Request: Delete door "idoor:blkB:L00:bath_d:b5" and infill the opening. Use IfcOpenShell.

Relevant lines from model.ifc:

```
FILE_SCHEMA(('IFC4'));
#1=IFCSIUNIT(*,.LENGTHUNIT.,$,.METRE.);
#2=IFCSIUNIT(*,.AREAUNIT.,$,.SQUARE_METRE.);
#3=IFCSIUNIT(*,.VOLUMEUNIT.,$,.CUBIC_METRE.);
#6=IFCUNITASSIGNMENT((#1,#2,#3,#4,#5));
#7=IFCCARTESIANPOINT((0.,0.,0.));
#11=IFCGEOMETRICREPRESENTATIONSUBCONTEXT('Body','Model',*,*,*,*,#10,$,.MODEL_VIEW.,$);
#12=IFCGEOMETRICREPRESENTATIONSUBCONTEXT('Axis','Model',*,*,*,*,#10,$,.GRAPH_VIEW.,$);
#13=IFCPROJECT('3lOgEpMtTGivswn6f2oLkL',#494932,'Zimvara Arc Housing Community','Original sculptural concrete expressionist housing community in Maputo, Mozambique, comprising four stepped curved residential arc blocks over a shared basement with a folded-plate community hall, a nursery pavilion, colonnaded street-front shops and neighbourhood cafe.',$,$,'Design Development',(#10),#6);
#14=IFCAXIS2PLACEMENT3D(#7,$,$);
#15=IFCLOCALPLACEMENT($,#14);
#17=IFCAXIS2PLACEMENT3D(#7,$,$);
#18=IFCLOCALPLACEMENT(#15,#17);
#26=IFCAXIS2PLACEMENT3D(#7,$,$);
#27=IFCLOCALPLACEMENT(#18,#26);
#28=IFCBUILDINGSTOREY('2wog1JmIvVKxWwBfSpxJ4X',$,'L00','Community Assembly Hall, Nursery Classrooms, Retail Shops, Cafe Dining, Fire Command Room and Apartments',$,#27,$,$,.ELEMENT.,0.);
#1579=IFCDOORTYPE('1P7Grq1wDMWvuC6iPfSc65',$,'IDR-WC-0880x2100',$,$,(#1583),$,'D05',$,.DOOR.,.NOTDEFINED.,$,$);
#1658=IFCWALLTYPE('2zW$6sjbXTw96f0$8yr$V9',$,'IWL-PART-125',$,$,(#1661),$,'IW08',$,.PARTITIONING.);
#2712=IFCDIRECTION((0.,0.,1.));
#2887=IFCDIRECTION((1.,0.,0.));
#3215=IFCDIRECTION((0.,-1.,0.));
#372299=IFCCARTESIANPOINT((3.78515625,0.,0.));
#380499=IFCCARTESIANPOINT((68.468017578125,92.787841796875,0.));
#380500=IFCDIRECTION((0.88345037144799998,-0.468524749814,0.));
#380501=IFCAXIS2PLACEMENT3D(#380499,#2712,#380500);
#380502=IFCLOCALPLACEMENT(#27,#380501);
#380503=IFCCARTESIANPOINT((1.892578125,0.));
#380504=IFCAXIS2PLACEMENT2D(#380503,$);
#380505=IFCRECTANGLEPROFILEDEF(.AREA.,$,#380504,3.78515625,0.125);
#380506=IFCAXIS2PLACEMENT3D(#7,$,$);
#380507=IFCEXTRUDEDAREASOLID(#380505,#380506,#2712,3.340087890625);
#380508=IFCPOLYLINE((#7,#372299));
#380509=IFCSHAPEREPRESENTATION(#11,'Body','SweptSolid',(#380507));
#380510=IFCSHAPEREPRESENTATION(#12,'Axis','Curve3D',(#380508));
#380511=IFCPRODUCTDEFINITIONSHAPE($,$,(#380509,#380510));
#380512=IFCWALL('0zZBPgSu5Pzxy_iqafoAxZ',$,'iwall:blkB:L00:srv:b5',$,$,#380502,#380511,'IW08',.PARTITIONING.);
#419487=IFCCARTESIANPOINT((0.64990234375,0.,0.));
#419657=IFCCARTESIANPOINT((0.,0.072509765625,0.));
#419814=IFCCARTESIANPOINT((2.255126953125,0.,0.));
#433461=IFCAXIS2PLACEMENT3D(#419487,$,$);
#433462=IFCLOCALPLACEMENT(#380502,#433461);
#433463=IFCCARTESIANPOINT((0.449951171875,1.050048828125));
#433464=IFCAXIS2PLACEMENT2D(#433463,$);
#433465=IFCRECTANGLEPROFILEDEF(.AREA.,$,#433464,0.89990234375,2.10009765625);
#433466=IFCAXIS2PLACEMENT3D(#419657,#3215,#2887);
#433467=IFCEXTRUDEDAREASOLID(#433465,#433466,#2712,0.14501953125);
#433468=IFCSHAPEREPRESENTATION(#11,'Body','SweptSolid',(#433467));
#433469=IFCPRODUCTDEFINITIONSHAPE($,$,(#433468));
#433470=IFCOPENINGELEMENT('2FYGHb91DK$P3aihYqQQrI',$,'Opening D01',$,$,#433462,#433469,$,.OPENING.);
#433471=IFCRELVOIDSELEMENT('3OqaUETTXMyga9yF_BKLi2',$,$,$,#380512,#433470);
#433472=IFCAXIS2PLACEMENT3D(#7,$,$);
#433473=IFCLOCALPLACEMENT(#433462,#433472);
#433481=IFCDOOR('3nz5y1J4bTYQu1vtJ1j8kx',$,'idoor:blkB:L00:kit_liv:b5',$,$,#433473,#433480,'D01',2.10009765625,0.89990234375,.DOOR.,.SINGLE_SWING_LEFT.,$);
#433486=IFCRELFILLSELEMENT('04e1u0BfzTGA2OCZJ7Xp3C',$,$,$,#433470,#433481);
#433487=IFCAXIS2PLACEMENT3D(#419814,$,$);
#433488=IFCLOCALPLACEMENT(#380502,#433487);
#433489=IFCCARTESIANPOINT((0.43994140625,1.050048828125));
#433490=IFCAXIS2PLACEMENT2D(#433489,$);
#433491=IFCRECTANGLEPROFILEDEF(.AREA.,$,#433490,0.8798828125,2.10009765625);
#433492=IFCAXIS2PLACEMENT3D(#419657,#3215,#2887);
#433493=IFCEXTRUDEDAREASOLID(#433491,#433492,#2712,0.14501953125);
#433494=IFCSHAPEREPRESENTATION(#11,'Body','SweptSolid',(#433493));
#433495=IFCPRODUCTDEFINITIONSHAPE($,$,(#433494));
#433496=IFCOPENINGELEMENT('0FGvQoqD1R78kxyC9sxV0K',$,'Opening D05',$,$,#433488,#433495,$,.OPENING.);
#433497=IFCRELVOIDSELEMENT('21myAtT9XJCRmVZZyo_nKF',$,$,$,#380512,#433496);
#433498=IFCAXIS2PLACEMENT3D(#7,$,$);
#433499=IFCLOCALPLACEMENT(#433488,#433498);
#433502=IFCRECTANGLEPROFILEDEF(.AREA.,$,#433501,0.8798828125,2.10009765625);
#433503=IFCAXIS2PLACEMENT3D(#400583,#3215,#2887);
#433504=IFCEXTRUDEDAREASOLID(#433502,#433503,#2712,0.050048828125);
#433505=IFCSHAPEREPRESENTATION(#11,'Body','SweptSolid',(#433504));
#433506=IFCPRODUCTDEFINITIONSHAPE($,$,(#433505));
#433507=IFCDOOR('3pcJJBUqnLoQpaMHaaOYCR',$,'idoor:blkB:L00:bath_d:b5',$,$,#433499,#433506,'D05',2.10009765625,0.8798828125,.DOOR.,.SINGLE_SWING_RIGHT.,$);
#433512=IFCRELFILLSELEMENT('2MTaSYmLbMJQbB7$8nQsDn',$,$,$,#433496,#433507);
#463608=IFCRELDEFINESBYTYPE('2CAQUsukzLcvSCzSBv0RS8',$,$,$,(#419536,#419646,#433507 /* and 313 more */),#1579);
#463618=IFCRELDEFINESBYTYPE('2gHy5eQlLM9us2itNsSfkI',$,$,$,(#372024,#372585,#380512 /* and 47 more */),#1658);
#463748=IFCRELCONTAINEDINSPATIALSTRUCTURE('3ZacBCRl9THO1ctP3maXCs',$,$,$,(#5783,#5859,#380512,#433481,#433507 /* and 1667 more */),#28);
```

```python
import ifcopenshell
import ifcopenshell.api.feature
import ifcopenshell.api.root
import ifcopenshell.geom
import ifcopenshell.util.shape

model = ifcopenshell.open("model.ifc")
settings = ifcopenshell.geom.settings()


def volume(element):
    """Net volume in cubic metres, openings subtracted."""
    shape = ifcopenshell.geom.create_shape(settings, element)
    return ifcopenshell.util.shape.get_volume(shape.geometry)


door = model.by_guid("3pcJJBUqnLoQpaMHaaOYCR")
opening = door.FillsVoids[0].RelatingOpeningElement
wall = opening.VoidsElements[0].RelatingBuildingElement
before = volume(wall)

ifcopenshell.api.root.remove_product(model, product=door)
ifcopenshell.api.feature.remove_feature(model, feature=opening)

after = volume(wall)

print(f"wall volume {before:.3f} -> {after:.3f} m3")

model.write("model-out.ifc")
```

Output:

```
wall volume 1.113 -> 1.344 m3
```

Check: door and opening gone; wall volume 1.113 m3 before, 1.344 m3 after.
